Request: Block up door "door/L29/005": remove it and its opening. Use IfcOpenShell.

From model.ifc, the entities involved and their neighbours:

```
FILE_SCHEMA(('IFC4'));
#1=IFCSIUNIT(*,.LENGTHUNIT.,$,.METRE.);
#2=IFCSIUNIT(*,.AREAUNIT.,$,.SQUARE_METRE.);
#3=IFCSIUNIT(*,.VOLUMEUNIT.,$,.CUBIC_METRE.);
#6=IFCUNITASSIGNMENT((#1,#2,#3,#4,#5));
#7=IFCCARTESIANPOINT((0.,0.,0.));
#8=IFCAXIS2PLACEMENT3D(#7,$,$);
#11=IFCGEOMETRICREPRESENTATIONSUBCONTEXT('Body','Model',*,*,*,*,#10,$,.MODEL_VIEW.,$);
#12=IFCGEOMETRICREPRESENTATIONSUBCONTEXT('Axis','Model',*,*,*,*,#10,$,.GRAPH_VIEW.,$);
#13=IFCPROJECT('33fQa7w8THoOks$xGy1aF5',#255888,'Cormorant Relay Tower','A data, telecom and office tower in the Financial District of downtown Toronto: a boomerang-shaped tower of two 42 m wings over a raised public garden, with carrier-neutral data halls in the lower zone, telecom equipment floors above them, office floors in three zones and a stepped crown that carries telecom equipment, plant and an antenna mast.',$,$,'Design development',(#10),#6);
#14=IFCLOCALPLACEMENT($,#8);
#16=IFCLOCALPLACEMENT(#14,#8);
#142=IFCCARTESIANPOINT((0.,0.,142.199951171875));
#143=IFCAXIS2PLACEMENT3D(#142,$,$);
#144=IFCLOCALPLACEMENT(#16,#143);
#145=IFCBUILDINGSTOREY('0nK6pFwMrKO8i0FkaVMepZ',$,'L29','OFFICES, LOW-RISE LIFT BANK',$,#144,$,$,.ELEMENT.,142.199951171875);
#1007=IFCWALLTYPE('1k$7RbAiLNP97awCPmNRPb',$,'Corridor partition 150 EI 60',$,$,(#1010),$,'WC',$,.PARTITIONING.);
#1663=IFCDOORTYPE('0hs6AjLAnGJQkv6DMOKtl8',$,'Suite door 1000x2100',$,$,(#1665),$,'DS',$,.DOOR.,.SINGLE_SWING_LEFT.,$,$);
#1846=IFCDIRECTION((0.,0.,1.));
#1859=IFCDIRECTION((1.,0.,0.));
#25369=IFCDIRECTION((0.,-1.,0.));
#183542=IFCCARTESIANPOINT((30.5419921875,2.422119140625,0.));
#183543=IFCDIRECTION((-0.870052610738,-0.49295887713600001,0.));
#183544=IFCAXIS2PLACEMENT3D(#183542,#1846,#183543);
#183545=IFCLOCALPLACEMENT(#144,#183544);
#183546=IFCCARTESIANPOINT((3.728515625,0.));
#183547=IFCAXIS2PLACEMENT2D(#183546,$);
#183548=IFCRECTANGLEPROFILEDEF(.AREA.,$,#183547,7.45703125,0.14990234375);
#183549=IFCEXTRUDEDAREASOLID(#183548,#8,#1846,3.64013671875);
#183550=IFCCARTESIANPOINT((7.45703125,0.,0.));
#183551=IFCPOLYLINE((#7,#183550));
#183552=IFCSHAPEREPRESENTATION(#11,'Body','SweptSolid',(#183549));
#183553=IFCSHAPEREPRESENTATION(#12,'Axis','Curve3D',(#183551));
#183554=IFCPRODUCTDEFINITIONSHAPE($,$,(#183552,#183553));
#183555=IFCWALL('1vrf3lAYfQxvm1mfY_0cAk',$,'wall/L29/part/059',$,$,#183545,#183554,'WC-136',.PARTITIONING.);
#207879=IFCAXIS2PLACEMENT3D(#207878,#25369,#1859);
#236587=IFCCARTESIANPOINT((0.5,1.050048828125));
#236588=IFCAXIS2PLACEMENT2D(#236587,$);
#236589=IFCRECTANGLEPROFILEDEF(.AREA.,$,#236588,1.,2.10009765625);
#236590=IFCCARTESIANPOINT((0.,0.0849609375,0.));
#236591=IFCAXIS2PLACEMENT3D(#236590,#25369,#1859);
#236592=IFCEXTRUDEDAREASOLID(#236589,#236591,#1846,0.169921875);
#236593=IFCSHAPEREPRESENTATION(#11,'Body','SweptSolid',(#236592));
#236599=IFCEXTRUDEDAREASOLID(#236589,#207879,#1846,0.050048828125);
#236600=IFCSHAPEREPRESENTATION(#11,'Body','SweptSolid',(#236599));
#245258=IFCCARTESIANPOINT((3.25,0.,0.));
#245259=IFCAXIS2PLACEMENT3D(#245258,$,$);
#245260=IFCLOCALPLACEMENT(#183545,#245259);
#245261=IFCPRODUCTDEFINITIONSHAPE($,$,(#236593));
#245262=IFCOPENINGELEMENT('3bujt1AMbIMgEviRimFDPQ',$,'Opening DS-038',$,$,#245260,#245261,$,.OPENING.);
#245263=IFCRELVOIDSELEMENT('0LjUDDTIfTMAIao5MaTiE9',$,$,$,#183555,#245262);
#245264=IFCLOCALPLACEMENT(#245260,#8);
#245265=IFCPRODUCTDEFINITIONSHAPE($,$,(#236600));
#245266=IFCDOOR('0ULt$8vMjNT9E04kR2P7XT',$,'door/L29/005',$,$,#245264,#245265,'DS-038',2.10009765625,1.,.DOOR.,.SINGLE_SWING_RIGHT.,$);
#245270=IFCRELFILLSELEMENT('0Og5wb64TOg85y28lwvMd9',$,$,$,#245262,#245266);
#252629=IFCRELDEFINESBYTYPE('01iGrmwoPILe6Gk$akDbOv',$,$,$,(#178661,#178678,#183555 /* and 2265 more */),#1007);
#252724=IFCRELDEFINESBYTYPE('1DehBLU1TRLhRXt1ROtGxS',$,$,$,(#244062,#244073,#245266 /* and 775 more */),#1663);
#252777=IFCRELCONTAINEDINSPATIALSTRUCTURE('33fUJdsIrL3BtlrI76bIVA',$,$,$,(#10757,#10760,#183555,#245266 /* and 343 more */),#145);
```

```python
import ifcopenshell
import ifcopenshell.api.feature
import ifcopenshell.api.root
import ifcopenshell.geom
import ifcopenshell.util.shape

model = ifcopenshell.open("model.ifc")
settings = ifcopenshell.geom.settings()


def volume(element):
    """Net volume in cubic metres, openings subtracted."""
    shape = ifcopenshell.geom.create_shape(settings, element)
    return ifcopenshell.util.shape.get_volume(shape.geometry)


door = model.by_guid("0ULt$8vMjNT9E04kR2P7XT")
opening = door.FillsVoids[0].RelatingOpeningElement
wall = opening.VoidsElements[0].RelatingBuildingElement
before = volume(wall)

ifcopenshell.api.root.remove_product(model, product=door)
ifcopenshell.api.feature.remove_feature(model, feature=opening)

after = volume(wall)

print(f"wall volume {before:.3f} -> {after:.3f} m3")

model.write("model_updated.ifc")
```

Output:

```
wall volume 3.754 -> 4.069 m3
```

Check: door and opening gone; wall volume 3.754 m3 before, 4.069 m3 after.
